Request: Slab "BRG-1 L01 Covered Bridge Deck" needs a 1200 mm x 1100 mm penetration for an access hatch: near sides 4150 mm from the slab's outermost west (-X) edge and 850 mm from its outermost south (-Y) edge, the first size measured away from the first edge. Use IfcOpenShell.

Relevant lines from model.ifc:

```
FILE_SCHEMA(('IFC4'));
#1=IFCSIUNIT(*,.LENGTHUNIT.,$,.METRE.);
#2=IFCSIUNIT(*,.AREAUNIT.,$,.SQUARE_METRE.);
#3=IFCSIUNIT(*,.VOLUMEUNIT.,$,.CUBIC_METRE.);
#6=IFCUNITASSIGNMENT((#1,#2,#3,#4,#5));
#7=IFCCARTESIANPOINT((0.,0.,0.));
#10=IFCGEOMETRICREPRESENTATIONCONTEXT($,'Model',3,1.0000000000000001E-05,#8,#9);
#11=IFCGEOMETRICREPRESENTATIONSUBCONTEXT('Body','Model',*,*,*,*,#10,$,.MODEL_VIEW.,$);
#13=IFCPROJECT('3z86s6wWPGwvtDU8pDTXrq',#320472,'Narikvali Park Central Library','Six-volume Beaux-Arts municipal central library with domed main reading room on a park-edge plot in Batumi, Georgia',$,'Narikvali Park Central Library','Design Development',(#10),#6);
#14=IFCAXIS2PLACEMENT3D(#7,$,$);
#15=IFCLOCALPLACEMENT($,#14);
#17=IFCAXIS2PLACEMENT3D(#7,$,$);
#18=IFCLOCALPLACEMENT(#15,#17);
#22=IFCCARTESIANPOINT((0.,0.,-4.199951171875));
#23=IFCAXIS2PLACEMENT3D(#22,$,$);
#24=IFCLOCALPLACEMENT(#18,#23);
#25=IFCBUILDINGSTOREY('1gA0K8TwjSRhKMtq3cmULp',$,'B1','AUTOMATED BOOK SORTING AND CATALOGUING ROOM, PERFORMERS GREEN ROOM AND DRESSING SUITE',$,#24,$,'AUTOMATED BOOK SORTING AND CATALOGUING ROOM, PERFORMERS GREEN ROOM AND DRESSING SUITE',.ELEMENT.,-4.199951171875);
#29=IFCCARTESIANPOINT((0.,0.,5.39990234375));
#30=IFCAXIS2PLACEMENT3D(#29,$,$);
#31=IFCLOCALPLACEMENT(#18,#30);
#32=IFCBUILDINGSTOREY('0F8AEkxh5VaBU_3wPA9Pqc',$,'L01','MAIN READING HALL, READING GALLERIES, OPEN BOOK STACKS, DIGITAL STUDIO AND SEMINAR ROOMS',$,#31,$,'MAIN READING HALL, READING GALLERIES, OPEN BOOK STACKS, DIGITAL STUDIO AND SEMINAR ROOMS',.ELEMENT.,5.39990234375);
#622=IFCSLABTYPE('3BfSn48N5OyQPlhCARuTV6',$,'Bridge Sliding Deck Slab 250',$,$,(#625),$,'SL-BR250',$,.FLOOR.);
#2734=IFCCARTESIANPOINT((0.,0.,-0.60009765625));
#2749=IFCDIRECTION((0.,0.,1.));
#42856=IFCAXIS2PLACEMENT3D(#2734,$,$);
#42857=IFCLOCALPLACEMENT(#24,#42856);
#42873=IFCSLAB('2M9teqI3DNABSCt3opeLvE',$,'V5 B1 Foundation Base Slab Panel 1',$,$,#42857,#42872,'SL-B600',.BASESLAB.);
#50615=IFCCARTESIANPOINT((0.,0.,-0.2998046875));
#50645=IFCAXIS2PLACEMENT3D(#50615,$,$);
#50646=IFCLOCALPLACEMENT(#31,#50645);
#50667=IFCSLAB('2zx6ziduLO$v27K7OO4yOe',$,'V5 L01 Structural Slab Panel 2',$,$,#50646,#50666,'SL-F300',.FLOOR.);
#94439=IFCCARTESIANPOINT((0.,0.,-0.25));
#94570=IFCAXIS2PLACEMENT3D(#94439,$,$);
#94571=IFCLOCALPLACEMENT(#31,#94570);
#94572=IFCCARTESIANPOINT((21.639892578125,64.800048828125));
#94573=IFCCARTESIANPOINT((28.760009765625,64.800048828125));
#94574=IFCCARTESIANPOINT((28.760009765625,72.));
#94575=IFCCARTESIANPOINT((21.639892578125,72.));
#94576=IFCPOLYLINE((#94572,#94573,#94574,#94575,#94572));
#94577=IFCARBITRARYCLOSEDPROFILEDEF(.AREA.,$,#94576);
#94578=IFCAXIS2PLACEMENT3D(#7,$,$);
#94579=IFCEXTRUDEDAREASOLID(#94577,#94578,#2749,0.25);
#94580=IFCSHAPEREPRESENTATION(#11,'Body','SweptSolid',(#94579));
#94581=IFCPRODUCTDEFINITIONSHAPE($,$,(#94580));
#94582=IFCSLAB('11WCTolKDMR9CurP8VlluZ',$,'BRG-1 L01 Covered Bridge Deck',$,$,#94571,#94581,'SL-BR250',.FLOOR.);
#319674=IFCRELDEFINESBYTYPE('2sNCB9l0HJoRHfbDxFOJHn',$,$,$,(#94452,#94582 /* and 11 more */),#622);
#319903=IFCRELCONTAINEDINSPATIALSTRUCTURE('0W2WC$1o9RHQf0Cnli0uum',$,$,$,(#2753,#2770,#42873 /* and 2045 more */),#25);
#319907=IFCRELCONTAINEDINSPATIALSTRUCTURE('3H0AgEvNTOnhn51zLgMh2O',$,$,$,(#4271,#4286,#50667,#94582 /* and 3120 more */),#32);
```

```python
import numpy as np
import ifcopenshell
import ifcopenshell.api.feature
import ifcopenshell.api.geometry
import ifcopenshell.api.root
import ifcopenshell.geom
import ifcopenshell.util.placement
import ifcopenshell.util.representation
import ifcopenshell.util.shape
import ifcopenshell.util.unit

model = ifcopenshell.open("model.ifc")
unit_scale = ifcopenshell.util.unit.calculate_unit_scale(model)
settings = ifcopenshell.geom.settings()


def volume(element):
    """Net volume in cubic metres, openings subtracted."""
    shape = ifcopenshell.geom.create_shape(settings, element)
    return ifcopenshell.util.shape.get_volume(shape.geometry)


slab = model.by_guid("11WCTolKDMR9CurP8VlluZ")
before = volume(slab)

# Extent in the slab's own axes, in metres. The edges named are its -X and -Y sides.
slab_shape = ifcopenshell.geom.create_shape(settings, slab)
vertices = ifcopenshell.util.shape.get_vertices(slab_shape.geometry)
x_min, y_min, bottom = vertices.min(axis=0)
top = vertices[:, 2].max()

opening = ifcopenshell.api.root.create_entity(model, ifc_class="IfcOpeningElement", name="Access hatch opening", predefined_type="OPENING")
context = ifcopenshell.util.representation.get_context(model, "Model", "Body", "MODEL_VIEW")
width, depth = 1.2, 1.1
outline = [(0.0, 0.0), (width, 0.0), (width, depth), (0.0, depth), (0.0, 0.0)]
# Overshoot both faces by 50 mm so the cut is clean.
shape = ifcopenshell.api.geometry.add_slab_representation(
    model, context=context, depth=top - bottom + 0.1, polyline=outline
)
ifcopenshell.api.geometry.assign_representation(model, product=opening, representation=shape)

matrix = ifcopenshell.util.placement.get_local_placement(slab.ObjectPlacement)
matrix[:, 3] = matrix @ np.append(np.array([x_min + 4.15, y_min + 0.85, bottom - 0.05]) / unit_scale, 1.0)
ifcopenshell.api.geometry.edit_object_placement(model, product=opening, matrix=matrix, is_si=False)
ifcopenshell.api.feature.add_feature(model, feature=opening, element=slab)

after = volume(slab)

print(f"slab volume {before:.3f} -> {after:.3f} m3")

model.write("model_updated.ifc")
```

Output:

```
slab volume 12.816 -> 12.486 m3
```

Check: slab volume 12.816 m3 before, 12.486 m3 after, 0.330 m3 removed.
